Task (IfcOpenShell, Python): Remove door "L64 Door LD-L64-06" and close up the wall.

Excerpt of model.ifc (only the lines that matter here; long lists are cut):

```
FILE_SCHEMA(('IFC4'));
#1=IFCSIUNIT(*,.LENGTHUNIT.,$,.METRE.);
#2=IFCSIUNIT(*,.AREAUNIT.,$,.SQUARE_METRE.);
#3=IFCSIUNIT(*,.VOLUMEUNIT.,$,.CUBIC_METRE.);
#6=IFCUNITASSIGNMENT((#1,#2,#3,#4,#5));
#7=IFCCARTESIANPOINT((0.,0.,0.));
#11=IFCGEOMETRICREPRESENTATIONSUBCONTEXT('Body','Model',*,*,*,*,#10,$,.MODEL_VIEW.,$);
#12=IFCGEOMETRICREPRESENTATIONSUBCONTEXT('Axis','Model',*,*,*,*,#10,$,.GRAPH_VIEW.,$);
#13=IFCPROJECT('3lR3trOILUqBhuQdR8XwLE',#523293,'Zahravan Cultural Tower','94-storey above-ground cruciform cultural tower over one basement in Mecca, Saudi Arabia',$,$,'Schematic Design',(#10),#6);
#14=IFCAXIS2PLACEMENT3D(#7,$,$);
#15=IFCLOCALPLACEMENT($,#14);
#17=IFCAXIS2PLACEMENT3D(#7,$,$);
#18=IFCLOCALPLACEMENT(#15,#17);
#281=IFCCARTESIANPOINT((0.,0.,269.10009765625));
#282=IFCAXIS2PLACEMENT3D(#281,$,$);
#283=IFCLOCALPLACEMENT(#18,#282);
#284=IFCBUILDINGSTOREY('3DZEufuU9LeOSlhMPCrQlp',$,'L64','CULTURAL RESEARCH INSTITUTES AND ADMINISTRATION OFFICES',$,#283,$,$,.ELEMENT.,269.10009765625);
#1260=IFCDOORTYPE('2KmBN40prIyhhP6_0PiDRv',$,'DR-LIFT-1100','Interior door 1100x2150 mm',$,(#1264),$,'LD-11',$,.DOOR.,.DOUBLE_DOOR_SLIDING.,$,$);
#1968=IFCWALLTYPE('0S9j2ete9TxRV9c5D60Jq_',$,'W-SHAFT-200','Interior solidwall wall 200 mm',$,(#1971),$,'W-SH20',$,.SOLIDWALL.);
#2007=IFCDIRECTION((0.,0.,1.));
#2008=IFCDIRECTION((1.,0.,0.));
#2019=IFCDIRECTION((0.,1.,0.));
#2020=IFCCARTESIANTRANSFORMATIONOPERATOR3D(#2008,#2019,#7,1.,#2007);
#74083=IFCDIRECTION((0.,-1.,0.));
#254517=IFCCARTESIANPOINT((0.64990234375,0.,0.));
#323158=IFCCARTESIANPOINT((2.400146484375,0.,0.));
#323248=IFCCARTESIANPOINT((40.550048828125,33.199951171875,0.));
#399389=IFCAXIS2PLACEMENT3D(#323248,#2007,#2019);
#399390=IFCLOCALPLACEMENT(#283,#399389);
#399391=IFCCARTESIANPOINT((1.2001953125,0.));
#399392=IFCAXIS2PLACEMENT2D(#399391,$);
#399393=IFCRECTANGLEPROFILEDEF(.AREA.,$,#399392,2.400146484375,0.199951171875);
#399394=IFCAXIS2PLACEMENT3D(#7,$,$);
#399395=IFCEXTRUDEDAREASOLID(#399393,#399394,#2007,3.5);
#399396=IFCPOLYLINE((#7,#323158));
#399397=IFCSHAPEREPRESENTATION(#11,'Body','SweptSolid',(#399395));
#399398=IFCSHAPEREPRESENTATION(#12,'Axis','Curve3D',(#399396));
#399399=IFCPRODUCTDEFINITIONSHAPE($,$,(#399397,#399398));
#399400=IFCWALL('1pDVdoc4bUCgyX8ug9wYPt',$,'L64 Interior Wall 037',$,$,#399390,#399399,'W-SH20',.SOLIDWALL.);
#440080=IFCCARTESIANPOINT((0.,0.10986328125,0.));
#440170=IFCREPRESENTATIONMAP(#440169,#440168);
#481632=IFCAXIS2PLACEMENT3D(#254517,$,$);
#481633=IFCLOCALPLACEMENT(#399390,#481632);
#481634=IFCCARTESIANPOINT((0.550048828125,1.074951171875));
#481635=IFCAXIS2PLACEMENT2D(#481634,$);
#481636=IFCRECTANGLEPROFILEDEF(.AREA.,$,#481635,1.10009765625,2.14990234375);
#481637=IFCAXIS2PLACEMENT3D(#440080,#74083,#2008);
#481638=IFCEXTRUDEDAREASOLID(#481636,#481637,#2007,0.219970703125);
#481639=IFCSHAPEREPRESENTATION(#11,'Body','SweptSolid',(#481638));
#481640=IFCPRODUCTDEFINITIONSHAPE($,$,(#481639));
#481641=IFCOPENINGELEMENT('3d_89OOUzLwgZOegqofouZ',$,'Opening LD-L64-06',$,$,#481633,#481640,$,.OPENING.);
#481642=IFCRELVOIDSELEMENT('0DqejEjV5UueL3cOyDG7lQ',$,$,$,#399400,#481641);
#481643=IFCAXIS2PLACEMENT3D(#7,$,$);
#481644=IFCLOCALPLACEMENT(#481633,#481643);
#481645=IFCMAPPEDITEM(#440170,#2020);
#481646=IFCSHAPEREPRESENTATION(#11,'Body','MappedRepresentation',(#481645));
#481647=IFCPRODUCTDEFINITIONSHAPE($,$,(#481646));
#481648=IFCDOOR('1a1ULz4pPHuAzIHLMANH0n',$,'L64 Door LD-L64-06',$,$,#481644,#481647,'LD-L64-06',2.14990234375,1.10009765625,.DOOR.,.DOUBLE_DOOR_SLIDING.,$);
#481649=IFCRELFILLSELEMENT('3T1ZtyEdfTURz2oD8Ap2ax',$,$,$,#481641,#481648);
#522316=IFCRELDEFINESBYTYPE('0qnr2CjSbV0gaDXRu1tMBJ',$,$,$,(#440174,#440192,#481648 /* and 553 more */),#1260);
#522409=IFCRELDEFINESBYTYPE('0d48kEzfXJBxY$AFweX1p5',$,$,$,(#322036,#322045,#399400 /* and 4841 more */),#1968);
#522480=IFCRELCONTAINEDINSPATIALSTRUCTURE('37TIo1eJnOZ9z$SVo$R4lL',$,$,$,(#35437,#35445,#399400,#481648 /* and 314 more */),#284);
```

```python
import ifcopenshell
import ifcopenshell.api.feature
import ifcopenshell.api.root
import ifcopenshell.geom
import ifcopenshell.util.shape

model = ifcopenshell.open("model.ifc")
settings = ifcopenshell.geom.settings()


def volume(element):
    """Net volume in cubic metres, openings subtracted."""
    shape = ifcopenshell.geom.create_shape(settings, element)
    return ifcopenshell.util.shape.get_volume(shape.geometry)


door = model.by_guid("1a1ULz4pPHuAzIHLMANH0n")
opening = door.FillsVoids[0].RelatingOpeningElement
wall = opening.VoidsElements[0].RelatingBuildingElement
before = volume(wall)

ifcopenshell.api.root.remove_product(model, product=door)
ifcopenshell.api.feature.remove_feature(model, feature=opening)

after = volume(wall)

print(f"wall volume {before:.3f} -> {after:.3f} m3")

model.write("model-out.ifc")
```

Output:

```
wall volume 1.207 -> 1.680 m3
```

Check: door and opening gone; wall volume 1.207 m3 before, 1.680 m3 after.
